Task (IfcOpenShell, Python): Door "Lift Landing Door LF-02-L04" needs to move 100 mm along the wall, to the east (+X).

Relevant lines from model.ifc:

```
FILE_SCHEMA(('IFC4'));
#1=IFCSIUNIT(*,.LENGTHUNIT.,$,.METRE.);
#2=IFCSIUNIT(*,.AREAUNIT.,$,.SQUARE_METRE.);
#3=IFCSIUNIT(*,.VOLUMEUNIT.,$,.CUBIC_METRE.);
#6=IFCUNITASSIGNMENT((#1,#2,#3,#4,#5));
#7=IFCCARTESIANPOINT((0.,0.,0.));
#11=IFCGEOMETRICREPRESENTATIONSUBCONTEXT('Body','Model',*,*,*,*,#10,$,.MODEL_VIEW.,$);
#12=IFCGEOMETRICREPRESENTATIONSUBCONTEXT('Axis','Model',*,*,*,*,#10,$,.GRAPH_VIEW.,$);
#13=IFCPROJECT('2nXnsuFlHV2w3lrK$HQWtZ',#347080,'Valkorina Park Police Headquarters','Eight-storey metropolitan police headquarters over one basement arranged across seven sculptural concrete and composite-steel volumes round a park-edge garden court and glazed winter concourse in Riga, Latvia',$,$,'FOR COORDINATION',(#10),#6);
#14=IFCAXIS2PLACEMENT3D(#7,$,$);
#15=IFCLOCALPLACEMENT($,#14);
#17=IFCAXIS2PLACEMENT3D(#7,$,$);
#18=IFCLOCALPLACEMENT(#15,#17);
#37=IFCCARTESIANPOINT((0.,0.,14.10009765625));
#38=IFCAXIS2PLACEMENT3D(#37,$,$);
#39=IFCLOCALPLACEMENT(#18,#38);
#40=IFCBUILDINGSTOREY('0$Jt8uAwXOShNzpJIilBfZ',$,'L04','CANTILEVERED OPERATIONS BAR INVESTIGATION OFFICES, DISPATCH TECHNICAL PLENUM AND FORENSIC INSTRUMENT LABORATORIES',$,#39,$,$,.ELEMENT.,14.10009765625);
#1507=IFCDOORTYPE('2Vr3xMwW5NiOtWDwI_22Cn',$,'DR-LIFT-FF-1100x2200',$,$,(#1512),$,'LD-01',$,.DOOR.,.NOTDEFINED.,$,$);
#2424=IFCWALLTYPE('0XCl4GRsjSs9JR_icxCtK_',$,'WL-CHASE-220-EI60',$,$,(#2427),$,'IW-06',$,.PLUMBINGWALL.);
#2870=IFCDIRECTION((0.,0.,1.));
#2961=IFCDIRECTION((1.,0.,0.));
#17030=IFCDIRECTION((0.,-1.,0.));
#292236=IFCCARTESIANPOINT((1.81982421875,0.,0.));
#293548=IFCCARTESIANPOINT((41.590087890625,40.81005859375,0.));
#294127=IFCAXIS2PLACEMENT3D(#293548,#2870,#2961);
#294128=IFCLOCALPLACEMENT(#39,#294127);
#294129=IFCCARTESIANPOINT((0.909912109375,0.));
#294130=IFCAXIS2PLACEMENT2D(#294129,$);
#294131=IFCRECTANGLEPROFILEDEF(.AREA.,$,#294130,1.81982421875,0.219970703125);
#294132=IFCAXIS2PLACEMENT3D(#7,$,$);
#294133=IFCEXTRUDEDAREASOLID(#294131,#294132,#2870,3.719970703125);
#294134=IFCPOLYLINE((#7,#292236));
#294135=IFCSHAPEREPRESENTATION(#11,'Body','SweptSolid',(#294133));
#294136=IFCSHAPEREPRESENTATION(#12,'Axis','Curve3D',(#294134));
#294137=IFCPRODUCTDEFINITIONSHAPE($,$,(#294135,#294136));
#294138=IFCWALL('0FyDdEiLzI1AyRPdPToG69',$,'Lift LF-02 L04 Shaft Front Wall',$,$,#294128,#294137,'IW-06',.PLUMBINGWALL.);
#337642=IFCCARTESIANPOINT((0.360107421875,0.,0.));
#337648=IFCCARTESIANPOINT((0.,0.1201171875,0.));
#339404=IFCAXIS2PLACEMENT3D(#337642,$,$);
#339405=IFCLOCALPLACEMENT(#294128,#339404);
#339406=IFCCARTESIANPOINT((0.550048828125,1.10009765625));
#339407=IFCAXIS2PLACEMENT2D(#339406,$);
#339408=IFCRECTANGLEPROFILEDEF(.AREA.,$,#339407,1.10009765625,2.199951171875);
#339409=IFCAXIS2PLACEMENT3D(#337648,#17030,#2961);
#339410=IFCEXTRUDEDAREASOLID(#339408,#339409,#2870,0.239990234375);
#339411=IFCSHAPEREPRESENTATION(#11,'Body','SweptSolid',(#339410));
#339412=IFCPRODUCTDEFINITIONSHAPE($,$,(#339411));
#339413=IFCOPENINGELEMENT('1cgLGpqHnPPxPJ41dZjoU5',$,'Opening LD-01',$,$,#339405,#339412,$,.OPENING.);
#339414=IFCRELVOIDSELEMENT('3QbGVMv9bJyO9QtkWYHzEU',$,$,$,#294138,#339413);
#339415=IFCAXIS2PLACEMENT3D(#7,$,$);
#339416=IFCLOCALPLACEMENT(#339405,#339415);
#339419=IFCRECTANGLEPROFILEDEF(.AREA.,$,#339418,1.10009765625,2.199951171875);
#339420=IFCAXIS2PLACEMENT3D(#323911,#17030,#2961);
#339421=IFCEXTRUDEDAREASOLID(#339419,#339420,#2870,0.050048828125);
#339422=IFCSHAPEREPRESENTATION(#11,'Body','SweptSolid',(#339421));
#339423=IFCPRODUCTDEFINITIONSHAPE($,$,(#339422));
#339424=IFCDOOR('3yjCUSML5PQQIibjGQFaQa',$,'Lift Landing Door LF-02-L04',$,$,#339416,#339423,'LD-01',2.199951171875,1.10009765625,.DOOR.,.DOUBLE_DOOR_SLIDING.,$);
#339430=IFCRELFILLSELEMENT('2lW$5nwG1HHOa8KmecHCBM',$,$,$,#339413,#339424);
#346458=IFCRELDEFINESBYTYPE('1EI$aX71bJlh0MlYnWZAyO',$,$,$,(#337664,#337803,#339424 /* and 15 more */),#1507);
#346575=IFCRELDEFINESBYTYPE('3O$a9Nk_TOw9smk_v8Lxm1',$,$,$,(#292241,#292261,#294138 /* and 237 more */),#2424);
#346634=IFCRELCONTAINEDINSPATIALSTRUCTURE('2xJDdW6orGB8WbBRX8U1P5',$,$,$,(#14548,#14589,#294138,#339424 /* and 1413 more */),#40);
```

```python
import ifcopenshell
import ifcopenshell.api.geometry
import ifcopenshell.util.placement
import ifcopenshell.util.unit

model = ifcopenshell.open("model.ifc")
unit_scale = ifcopenshell.util.unit.calculate_unit_scale(model)

door = model.by_guid("3yjCUSML5PQQIibjGQFaQa")
opening = door.FillsVoids[0].RelatingOpeningElement
wall = opening.VoidsElements[0].RelatingBuildingElement

wall_matrix = ifcopenshell.util.placement.get_local_placement(wall.ObjectPlacement)
shift = wall_matrix[:3, 0] * 0.1 / unit_scale
before = ifcopenshell.util.placement.get_local_placement(door.ObjectPlacement)[:3, 3].copy()

# The door is placed relative to its opening, so it follows when the opening moves.
matrix = ifcopenshell.util.placement.get_local_placement(opening.ObjectPlacement)
matrix[:3, 3] += shift
ifcopenshell.api.geometry.edit_object_placement(
    model, product=opening, matrix=matrix, is_si=False, should_transform_children=True
)

after = ifcopenshell.util.placement.get_local_placement(door.ObjectPlacement)[:3, 3]
print("door moved by", (after - before).round(3) + 0.0)

model.write("model_v2.ifc")
```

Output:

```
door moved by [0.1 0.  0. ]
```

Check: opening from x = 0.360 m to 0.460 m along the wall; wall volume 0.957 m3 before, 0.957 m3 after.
